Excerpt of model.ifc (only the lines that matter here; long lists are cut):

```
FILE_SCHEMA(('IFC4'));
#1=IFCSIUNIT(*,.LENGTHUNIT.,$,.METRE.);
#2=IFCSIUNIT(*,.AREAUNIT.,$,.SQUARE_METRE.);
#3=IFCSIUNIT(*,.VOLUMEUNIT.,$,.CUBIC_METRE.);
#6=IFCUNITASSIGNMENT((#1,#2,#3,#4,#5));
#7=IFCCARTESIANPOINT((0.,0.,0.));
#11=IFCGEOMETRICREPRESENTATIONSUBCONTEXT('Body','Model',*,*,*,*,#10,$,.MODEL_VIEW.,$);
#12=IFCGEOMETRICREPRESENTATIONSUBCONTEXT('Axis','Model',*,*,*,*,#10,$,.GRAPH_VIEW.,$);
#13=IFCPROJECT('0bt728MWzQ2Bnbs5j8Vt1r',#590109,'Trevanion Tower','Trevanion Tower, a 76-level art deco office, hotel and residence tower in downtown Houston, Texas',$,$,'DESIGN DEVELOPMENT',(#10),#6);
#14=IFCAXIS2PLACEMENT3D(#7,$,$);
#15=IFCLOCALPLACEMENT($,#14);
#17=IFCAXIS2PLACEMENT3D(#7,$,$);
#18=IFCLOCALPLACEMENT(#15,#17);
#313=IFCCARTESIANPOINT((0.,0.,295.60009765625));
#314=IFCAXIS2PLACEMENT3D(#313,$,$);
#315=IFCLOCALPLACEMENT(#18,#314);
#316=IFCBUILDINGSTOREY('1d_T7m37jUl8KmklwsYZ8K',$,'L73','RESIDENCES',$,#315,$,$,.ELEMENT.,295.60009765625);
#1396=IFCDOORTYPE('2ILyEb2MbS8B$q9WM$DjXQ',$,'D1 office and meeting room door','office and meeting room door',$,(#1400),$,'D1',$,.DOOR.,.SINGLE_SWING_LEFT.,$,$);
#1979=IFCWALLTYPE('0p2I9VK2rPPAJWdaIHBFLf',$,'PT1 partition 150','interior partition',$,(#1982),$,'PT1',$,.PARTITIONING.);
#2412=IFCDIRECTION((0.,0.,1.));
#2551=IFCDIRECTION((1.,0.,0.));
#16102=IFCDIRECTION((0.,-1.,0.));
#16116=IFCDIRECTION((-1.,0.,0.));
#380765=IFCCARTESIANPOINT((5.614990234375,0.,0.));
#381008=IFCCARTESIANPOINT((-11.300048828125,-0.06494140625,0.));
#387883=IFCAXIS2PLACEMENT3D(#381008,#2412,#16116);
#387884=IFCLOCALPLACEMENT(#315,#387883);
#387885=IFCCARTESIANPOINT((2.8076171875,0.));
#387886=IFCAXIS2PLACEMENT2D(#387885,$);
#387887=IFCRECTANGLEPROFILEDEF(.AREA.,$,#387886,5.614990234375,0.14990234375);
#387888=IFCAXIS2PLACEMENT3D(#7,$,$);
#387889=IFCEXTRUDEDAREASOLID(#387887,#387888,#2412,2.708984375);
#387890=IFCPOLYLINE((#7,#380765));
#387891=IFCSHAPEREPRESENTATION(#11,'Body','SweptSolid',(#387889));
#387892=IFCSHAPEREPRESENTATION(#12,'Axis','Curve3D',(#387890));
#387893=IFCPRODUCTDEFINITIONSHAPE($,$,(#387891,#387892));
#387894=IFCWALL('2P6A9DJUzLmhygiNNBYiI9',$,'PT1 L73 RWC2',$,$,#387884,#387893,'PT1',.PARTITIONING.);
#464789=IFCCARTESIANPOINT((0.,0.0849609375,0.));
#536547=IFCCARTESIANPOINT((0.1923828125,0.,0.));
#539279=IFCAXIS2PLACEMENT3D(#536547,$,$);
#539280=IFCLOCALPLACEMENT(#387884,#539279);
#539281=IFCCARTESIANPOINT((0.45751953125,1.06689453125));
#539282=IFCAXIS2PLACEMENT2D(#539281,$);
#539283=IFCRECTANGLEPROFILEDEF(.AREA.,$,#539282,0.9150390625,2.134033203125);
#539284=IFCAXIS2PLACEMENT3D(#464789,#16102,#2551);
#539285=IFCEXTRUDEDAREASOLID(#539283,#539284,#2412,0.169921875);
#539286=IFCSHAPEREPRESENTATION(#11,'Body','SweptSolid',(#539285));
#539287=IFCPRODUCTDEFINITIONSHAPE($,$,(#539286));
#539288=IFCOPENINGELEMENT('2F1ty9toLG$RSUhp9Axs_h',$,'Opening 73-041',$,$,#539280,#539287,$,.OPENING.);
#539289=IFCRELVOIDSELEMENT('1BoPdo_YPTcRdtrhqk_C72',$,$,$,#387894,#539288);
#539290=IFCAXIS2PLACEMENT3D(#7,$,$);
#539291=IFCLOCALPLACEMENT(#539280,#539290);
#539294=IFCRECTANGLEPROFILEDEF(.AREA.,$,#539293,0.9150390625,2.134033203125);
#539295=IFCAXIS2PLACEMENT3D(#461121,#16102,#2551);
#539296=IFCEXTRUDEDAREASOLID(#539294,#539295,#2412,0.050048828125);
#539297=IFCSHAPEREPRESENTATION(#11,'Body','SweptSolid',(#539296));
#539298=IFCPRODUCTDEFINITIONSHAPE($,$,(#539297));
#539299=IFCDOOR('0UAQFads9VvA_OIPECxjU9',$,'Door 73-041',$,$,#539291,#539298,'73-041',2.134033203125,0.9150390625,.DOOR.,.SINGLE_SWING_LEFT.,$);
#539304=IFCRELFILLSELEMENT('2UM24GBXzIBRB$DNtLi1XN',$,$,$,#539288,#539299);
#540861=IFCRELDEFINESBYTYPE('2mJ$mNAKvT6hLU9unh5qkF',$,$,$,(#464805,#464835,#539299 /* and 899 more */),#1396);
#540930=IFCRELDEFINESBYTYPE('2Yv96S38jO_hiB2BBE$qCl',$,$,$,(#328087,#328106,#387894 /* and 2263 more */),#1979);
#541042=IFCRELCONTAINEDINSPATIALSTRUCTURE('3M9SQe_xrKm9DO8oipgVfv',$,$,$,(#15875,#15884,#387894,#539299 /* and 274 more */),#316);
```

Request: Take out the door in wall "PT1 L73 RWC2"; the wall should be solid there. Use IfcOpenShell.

```python
import ifcopenshell
import ifcopenshell.api.feature
import ifcopenshell.api.root
import ifcopenshell.geom
import ifcopenshell.util.shape

model = ifcopenshell.open("model.ifc")
settings = ifcopenshell.geom.settings()


def volume(element):
    """Net volume in cubic metres, openings subtracted."""
    shape = ifcopenshell.geom.create_shape(settings, element)
    return ifcopenshell.util.shape.get_volume(shape.geometry)


door = model.by_id(539299)
opening = door.FillsVoids[0].RelatingOpeningElement
wall = opening.VoidsElements[0].RelatingBuildingElement
before = volume(wall)

ifcopenshell.api.root.remove_product(model, product=door)
ifcopenshell.api.feature.remove_feature(model, feature=opening)

after = volume(wall)

print(f"wall volume {before:.3f} -> {after:.3f} m3")

model.write("model-out.ifc")
```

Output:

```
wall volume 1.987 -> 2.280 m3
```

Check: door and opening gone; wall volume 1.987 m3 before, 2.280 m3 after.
